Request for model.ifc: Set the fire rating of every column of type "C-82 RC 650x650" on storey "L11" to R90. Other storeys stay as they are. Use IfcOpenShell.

First a look at what the model holds.

```python
import ifcopenshell
import ifcopenshell.util.element

model = ifcopenshell.open("model.ifc")
print(model.schema)
storey = next(s for s in model.by_type("IfcBuildingStorey") if s.Name == "L11")
columns = [e for e in ifcopenshell.util.element.get_decomposition(storey) if e.is_a("IfcColumn")]
seen = {}
for e in columns:
    element_type = ifcopenshell.util.element.get_type(e)
    key = (element_type.Name if element_type != e and element_type else None, ifcopenshell.util.element.get_pset(e, "Pset_ColumnCommon", "FireRating"))
    seen[key] = seen.get(key, 0) + 1
for (name, value), count in sorted(seen.items(), key=str):
    print(count, "x", name, "|", value)
```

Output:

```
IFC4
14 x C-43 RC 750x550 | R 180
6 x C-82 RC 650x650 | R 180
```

```python
import ifcopenshell
import ifcopenshell.api.pset
import ifcopenshell.util.element

model = ifcopenshell.open("model.ifc")

storey = next(s for s in model.by_type("IfcBuildingStorey") if s.Name == "L11")
columns = [e for e in ifcopenshell.util.element.get_decomposition(storey) if e.is_a("IfcColumn")]

count = 0
for e in columns:
    element_type = ifcopenshell.util.element.get_type(e)
    if element_type in (None, e) or element_type.Name != "C-82 RC 650x650":
        continue
    # add_pset returns the element's existing set when there is one.
    pset = ifcopenshell.api.pset.add_pset(model, product=e, name="Pset_ColumnCommon")
    ifcopenshell.api.pset.edit_pset(model, pset=pset, properties={"FireRating": "R90"})
    count += 1

print(count, "columns updated")

model.write("model-out.ifc")
```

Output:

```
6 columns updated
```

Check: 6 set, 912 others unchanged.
